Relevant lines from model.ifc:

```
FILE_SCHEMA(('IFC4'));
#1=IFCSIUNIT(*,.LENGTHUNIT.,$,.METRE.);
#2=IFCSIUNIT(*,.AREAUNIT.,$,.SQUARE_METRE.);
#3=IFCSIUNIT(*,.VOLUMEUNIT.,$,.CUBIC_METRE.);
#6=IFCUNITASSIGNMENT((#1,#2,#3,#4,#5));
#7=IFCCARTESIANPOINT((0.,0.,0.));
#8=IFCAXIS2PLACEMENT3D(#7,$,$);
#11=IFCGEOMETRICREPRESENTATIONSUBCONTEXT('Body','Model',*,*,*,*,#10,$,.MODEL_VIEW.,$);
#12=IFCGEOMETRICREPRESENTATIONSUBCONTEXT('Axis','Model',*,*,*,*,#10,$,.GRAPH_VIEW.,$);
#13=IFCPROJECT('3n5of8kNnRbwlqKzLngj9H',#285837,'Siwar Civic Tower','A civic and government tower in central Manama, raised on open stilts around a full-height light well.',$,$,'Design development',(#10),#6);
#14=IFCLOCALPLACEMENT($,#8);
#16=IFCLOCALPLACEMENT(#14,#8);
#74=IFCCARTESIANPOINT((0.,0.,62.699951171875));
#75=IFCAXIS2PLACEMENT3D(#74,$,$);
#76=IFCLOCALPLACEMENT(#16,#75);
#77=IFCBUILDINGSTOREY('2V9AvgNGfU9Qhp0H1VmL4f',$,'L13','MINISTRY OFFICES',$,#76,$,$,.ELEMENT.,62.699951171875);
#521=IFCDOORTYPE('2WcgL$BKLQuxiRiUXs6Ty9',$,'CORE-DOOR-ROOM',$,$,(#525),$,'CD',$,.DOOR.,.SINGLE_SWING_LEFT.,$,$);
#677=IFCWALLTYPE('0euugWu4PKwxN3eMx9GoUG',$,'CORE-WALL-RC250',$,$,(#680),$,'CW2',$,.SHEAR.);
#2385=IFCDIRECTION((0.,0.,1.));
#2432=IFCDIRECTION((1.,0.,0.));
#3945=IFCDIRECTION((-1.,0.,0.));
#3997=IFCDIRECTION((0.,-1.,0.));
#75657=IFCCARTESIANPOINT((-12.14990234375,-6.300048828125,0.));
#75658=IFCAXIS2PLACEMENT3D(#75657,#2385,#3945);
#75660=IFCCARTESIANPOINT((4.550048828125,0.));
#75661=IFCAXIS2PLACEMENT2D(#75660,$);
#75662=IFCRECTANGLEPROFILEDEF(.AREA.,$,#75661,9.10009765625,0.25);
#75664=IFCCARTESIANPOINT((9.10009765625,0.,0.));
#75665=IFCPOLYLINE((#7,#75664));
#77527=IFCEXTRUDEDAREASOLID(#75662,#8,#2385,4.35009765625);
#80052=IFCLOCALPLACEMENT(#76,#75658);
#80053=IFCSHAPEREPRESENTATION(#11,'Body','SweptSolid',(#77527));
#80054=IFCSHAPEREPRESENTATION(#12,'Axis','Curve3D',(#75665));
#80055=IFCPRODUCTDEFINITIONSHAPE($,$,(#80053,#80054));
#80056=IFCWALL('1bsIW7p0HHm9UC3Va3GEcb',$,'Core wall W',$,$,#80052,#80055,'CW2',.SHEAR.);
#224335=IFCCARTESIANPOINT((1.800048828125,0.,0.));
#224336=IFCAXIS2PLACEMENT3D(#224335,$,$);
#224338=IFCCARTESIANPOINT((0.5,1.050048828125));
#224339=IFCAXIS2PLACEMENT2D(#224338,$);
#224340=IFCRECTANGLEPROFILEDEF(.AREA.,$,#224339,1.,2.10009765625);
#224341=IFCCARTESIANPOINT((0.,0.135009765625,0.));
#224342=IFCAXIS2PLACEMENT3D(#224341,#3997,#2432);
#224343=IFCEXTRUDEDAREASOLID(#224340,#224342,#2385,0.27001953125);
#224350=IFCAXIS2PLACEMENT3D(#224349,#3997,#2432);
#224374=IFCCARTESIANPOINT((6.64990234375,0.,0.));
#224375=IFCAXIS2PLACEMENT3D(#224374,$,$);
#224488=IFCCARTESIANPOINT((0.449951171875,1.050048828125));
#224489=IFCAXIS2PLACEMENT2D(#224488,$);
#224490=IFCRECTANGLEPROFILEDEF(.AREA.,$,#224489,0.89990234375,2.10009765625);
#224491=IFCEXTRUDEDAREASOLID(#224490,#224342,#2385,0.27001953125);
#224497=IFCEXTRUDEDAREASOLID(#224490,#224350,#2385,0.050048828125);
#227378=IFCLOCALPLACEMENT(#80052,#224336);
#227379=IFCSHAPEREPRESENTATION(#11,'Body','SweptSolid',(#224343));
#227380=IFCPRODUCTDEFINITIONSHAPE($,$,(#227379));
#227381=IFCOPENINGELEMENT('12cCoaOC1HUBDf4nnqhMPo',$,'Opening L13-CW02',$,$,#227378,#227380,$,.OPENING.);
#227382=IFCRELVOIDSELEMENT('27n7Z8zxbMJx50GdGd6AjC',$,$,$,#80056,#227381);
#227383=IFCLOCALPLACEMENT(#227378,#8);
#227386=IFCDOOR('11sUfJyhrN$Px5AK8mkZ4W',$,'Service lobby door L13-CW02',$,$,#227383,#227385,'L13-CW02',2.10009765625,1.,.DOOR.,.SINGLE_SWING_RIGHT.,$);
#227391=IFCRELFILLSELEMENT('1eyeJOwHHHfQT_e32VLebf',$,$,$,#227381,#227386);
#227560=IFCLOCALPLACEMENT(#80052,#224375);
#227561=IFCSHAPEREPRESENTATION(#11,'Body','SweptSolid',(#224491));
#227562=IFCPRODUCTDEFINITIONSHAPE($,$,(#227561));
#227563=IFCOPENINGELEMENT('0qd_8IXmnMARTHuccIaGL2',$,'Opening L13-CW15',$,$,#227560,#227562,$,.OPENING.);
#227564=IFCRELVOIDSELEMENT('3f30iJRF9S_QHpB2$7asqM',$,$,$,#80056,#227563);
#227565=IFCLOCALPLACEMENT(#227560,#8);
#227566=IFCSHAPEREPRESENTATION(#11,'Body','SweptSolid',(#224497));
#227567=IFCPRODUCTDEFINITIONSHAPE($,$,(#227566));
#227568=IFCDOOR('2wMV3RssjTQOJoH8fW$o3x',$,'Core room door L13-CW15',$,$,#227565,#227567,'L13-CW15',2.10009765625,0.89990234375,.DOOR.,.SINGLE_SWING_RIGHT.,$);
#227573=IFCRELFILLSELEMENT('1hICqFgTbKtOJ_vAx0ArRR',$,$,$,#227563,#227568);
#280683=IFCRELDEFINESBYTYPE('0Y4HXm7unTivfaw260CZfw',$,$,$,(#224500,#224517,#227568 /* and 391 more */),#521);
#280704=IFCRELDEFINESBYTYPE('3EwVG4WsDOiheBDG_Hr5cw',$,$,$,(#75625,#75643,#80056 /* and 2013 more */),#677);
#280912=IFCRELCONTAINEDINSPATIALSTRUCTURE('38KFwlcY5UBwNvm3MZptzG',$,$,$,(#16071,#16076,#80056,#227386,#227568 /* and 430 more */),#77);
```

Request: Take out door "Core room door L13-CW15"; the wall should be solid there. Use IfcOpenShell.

```python
import ifcopenshell
import ifcopenshell.api.feature
import ifcopenshell.api.root
import ifcopenshell.geom
import ifcopenshell.util.shape

model = ifcopenshell.open("model.ifc")
settings = ifcopenshell.geom.settings()


def volume(element):
    """Net volume in cubic metres, openings subtracted."""
    shape = ifcopenshell.geom.create_shape(settings, element)
    return ifcopenshell.util.shape.get_volume(shape.geometry)


door = model.by_guid("2wMV3RssjTQOJoH8fW$o3x")
opening = door.FillsVoids[0].RelatingOpeningElement
wall = opening.VoidsElements[0].RelatingBuildingElement
before = volume(wall)

ifcopenshell.api.root.remove_product(model, product=door)
ifcopenshell.api.feature.remove_feature(model, feature=opening)

after = volume(wall)

print(f"wall volume {before:.3f} -> {after:.3f} m3")

model.write("model-out.ifc")
```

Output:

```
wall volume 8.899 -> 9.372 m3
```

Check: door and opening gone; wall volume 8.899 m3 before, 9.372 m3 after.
